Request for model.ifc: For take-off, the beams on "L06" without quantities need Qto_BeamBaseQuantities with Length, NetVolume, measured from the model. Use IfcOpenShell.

First a look at what the model holds.

```python
import ifcopenshell
import ifcopenshell.util.element
import ifcopenshell.util.unit

model = ifcopenshell.open("model.ifc")
print(model.schema)
for unit_type in ("LENGTHUNIT", "AREAUNIT", "VOLUMEUNIT"):
    print(unit_type, ifcopenshell.util.unit.calculate_unit_scale(model, unit_type))
storey = next(s for s in model.by_type("IfcBuildingStorey") if s.Name == "L06")
beams = [e for e in ifcopenshell.util.element.get_decomposition(storey) if e.is_a("IfcBeam")]
for e in sorted(beams, key=lambda e: e.id()):
    print(e.id(), e.is_a(), e.Name, list(ifcopenshell.util.element.get_psets(e, qtos_only=True)), sep=" | ")
```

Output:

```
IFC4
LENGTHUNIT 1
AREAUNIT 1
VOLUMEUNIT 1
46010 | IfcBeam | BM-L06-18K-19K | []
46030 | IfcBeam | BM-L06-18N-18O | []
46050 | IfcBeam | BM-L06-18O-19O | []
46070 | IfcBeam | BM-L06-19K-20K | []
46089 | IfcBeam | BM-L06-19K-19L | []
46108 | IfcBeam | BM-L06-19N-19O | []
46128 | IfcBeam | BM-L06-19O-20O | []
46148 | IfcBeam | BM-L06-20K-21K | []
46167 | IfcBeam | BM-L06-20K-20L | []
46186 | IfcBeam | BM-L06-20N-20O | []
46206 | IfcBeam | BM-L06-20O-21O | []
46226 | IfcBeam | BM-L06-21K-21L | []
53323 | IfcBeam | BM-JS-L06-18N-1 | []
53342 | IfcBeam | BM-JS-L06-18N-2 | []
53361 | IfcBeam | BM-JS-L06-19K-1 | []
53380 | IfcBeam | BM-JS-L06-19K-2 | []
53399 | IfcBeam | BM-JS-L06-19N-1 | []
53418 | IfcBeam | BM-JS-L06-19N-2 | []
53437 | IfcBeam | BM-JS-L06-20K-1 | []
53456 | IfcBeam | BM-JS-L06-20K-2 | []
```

```python
import ifcopenshell
import ifcopenshell.api.pset
import ifcopenshell.geom
import ifcopenshell.util.element
import ifcopenshell.util.shape
import ifcopenshell.util.unit

model = ifcopenshell.open("model.ifc")
unit_scale = ifcopenshell.util.unit.calculate_unit_scale(model)
volume_scale = ifcopenshell.util.unit.calculate_unit_scale(model, "VOLUMEUNIT")
settings = ifcopenshell.geom.settings()

storey = next(s for s in model.by_type("IfcBuildingStorey") if s.Name == "L06")
beams = [e for e in ifcopenshell.util.element.get_decomposition(storey) if e.is_a("IfcBeam")]

for e in sorted(beams, key=lambda e: e.id()):
    if ifcopenshell.util.element.get_psets(e, qtos_only=True, should_inherit=False):
        continue
    # Geometry comes back in metres, in the element's own axes.
    shape = ifcopenshell.geom.create_shape(settings, e)
    values = {
        "Length": ifcopenshell.util.shape.get_max_xyz(shape.geometry) / unit_scale,
        "NetVolume": ifcopenshell.util.shape.get_volume(shape.geometry) / volume_scale,
    }
    qto = ifcopenshell.api.pset.add_qto(model, product=e, name="Qto_BeamBaseQuantities")
    ifcopenshell.api.pset.edit_qto(model, qto=qto, properties=values)
    print(e.id(), {k: round(v, 3) for k, v in values.items()})

model.write("model-out.ifc")
```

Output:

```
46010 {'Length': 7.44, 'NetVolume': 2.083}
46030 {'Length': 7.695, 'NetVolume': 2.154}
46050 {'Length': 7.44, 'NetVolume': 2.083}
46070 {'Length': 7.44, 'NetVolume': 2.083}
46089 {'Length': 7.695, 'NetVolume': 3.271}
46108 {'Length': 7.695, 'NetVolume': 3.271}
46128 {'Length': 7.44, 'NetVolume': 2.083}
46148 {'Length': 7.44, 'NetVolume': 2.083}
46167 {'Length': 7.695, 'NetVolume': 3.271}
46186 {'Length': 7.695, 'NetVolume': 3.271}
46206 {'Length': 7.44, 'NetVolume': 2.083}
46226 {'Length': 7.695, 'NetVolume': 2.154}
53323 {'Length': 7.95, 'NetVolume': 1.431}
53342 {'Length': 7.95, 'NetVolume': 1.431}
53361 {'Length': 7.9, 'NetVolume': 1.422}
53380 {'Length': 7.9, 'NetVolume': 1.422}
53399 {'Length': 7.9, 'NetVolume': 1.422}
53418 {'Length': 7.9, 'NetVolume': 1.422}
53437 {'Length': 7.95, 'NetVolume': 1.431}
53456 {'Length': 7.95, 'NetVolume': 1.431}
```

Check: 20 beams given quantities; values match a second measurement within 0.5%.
